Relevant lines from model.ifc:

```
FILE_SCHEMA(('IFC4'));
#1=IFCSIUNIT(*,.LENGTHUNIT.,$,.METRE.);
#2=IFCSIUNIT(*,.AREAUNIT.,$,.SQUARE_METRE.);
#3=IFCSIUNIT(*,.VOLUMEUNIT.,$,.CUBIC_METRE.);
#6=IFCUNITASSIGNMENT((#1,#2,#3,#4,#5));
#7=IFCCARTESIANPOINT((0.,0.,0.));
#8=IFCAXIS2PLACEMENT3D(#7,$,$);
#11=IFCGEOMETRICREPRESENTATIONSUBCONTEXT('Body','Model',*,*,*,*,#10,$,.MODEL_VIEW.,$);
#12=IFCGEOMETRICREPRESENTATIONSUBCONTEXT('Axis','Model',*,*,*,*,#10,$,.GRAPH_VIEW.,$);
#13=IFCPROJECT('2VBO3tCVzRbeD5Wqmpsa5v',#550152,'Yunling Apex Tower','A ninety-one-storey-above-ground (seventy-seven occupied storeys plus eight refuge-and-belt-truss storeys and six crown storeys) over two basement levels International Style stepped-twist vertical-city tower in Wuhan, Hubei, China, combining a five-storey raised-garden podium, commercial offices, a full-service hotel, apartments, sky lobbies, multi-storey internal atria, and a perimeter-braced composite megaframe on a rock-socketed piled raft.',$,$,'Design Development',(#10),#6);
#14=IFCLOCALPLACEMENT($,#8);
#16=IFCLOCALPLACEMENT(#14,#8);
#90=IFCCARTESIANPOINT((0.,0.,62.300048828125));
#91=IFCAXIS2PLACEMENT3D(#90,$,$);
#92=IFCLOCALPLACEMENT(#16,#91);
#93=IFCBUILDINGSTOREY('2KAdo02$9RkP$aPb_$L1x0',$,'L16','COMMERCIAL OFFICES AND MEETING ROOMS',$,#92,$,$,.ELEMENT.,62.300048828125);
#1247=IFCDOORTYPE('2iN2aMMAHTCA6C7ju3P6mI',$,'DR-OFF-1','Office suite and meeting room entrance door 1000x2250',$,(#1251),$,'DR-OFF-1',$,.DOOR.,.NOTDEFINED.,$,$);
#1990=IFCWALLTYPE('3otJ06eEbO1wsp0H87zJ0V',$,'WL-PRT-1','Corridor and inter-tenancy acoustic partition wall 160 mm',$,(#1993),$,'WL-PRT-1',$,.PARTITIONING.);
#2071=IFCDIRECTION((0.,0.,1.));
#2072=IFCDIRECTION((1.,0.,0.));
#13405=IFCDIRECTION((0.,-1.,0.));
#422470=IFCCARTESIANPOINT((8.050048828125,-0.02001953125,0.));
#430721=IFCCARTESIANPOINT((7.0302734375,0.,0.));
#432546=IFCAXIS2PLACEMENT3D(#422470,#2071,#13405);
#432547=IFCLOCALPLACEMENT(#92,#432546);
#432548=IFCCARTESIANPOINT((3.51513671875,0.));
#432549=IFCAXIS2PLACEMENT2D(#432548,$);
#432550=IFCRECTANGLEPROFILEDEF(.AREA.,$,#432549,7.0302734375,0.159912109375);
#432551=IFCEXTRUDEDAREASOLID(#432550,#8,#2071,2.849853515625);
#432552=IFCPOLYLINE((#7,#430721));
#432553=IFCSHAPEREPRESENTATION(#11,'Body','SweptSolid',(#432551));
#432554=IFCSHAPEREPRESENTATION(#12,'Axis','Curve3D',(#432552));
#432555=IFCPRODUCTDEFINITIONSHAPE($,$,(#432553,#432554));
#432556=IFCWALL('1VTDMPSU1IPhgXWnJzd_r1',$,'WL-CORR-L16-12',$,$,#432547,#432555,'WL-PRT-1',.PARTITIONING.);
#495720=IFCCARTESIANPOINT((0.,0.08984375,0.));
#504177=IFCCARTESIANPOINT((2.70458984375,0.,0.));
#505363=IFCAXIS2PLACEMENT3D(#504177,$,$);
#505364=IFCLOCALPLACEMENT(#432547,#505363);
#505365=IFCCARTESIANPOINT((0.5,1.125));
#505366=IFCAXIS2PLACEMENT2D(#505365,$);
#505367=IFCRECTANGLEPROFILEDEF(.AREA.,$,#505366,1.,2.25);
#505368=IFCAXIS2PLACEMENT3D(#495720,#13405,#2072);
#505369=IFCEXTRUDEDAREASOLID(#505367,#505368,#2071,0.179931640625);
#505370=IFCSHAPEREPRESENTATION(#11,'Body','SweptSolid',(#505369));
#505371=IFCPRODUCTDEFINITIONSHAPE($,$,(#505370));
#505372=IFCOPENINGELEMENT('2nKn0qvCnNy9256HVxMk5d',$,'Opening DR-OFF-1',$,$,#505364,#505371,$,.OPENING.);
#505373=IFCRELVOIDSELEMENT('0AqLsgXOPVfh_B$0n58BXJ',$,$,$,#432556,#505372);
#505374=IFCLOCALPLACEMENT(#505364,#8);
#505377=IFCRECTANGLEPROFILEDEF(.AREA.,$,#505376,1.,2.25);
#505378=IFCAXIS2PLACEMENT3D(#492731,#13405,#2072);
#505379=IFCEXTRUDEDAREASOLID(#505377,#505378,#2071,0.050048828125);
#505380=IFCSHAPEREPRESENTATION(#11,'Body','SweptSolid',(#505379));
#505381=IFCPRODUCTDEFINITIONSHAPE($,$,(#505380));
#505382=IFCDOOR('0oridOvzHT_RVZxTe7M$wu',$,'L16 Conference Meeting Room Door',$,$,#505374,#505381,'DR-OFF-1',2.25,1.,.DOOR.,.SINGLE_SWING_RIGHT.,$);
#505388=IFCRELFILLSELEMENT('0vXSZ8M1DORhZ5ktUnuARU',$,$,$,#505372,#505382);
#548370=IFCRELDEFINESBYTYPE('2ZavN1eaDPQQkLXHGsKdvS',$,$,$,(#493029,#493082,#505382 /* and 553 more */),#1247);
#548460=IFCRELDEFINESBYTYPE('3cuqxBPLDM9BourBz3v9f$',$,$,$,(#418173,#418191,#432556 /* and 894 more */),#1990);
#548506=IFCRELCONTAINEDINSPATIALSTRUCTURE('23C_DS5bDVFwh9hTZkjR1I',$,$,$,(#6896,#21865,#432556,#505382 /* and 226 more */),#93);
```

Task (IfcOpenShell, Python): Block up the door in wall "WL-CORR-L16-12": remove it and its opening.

```python
import ifcopenshell
import ifcopenshell.api.feature
import ifcopenshell.api.root
import ifcopenshell.geom
import ifcopenshell.util.shape

model = ifcopenshell.open("model.ifc")
settings = ifcopenshell.geom.settings()


def volume(element):
    """Net volume in cubic metres, openings subtracted."""
    shape = ifcopenshell.geom.create_shape(settings, element)
    return ifcopenshell.util.shape.get_volume(shape.geometry)


door = model.by_guid("0oridOvzHT_RVZxTe7M$wu")
opening = door.FillsVoids[0].RelatingOpeningElement
wall = opening.VoidsElements[0].RelatingBuildingElement
before = volume(wall)

ifcopenshell.api.root.remove_product(model, product=door)
ifcopenshell.api.feature.remove_feature(model, feature=opening)

after = volume(wall)

print(f"wall volume {before:.3f} -> {after:.3f} m3")

model.write("model_edited.ifc")
```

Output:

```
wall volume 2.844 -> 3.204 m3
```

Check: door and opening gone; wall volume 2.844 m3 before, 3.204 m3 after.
